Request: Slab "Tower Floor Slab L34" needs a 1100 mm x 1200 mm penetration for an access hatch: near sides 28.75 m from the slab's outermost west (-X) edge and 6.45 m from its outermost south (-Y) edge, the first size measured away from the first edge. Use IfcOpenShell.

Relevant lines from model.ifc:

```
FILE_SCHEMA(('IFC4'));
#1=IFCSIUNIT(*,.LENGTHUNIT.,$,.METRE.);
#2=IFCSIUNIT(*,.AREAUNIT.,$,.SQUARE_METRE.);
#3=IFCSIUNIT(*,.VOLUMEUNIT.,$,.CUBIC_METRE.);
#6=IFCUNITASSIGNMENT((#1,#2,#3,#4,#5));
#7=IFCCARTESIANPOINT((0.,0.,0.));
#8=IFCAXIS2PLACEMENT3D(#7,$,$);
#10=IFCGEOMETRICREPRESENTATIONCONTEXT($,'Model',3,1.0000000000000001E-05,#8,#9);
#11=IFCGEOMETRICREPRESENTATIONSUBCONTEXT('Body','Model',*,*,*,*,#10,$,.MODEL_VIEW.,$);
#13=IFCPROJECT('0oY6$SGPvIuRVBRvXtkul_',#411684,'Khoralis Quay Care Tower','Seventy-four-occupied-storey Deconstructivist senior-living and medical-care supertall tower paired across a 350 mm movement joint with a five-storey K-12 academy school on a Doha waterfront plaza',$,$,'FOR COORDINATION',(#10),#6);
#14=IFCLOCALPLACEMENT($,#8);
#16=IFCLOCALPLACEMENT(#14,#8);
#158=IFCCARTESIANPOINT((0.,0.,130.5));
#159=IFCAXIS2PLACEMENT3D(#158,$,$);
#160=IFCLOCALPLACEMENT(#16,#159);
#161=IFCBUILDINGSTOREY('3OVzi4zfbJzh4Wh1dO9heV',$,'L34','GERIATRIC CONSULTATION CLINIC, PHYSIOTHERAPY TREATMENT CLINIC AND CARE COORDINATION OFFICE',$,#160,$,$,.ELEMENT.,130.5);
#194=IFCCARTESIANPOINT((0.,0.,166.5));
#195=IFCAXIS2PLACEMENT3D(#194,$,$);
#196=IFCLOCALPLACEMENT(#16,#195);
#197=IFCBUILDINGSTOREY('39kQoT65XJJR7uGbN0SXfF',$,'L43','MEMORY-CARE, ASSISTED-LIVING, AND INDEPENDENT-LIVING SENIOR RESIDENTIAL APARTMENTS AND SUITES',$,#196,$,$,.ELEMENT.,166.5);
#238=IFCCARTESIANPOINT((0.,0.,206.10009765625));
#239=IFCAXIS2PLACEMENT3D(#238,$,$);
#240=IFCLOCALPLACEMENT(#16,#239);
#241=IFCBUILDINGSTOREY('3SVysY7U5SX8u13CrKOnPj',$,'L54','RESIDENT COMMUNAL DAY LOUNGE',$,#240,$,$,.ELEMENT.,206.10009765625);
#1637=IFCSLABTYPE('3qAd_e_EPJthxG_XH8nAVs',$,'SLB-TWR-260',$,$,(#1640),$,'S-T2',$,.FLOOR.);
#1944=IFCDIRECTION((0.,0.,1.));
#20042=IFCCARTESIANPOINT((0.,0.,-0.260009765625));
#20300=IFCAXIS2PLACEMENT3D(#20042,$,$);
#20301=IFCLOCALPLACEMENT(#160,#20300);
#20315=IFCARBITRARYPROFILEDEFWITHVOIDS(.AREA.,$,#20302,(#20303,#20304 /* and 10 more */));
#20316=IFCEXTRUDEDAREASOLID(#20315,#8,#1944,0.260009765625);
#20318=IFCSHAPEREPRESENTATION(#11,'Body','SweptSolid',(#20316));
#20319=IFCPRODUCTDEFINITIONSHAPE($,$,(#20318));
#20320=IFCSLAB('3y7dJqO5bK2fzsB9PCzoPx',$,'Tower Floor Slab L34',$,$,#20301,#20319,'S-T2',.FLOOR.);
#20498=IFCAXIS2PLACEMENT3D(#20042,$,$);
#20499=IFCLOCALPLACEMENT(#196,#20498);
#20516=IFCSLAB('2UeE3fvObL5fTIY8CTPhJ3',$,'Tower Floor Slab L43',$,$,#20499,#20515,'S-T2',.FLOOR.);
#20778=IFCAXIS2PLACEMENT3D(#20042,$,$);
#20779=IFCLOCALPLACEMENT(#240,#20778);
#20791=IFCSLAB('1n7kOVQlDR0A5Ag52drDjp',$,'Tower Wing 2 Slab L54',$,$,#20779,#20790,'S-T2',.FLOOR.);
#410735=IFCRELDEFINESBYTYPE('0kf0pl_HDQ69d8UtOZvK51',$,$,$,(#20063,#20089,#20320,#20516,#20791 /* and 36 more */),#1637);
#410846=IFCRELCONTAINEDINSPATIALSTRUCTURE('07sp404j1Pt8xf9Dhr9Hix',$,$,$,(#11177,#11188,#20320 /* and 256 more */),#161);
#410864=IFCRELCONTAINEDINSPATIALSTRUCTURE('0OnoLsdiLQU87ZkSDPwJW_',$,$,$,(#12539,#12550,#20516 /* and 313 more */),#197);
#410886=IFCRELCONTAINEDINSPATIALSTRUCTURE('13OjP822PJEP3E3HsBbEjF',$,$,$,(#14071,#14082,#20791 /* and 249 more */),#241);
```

```python
import numpy as np
import ifcopenshell
import ifcopenshell.api.feature
import ifcopenshell.api.geometry
import ifcopenshell.api.root
import ifcopenshell.geom
import ifcopenshell.util.placement
import ifcopenshell.util.representation
import ifcopenshell.util.shape
import ifcopenshell.util.unit

model = ifcopenshell.open("model.ifc")
unit_scale = ifcopenshell.util.unit.calculate_unit_scale(model)
settings = ifcopenshell.geom.settings()


def volume(element):
    """Net volume in cubic metres, openings subtracted."""
    shape = ifcopenshell.geom.create_shape(settings, element)
    return ifcopenshell.util.shape.get_volume(shape.geometry)


slab = model.by_guid("3y7dJqO5bK2fzsB9PCzoPx")
before = volume(slab)

# Extent in the slab's own axes, in metres. The edges named are its -X and -Y sides.
slab_shape = ifcopenshell.geom.create_shape(settings, slab)
vertices = ifcopenshell.util.shape.get_vertices(slab_shape.geometry)
x_min, y_min, bottom = vertices.min(axis=0)
top = vertices[:, 2].max()

opening = ifcopenshell.api.root.create_entity(model, ifc_class="IfcOpeningElement", name="Access hatch opening", predefined_type="OPENING")
context = ifcopenshell.util.representation.get_context(model, "Model", "Body", "MODEL_VIEW")
width, depth = 1.1, 1.2
outline = [(0.0, 0.0), (width, 0.0), (width, depth), (0.0, depth), (0.0, 0.0)]
# Overshoot both faces by 50 mm so the cut is clean.
shape = ifcopenshell.api.geometry.add_slab_representation(
    model, context=context, depth=top - bottom + 0.1, polyline=outline
)
ifcopenshell.api.geometry.assign_representation(model, product=opening, representation=shape)

matrix = ifcopenshell.util.placement.get_local_placement(slab.ObjectPlacement)
matrix[:, 3] = matrix @ np.append(np.array([x_min + 28.75, y_min + 6.45, bottom - 0.05]) / unit_scale, 1.0)
ifcopenshell.api.geometry.edit_object_placement(model, product=opening, matrix=matrix, is_si=False)
ifcopenshell.api.feature.add_feature(model, feature=opening, element=slab)

after = volume(slab)

print(f"slab volume {before:.3f} -> {after:.3f} m3")

model.write("model-out.ifc")
```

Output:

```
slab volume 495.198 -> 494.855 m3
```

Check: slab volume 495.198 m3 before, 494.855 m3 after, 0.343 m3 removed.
